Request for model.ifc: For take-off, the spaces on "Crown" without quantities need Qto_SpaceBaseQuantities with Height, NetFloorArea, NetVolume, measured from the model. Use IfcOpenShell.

First a look at what the model holds.

```python
import ifcopenshell
import ifcopenshell.util.element
import ifcopenshell.util.unit

model = ifcopenshell.open("model.ifc")
print(model.schema)
for unit_type in ("LENGTHUNIT", "AREAUNIT", "VOLUMEUNIT"):
    print(unit_type, ifcopenshell.util.unit.calculate_unit_scale(model, unit_type))
storey = next(s for s in model.by_type("IfcBuildingStorey") if s.Name == "Crown")
spaces = [e for e in ifcopenshell.util.element.get_decomposition(storey) if e.is_a("IfcSpace")]
for e in sorted(spaces, key=lambda e: e.id()):
    print(e.id(), e.is_a(), e.Name, list(ifcopenshell.util.element.get_psets(e, qtos_only=True)), sep=" | ")
```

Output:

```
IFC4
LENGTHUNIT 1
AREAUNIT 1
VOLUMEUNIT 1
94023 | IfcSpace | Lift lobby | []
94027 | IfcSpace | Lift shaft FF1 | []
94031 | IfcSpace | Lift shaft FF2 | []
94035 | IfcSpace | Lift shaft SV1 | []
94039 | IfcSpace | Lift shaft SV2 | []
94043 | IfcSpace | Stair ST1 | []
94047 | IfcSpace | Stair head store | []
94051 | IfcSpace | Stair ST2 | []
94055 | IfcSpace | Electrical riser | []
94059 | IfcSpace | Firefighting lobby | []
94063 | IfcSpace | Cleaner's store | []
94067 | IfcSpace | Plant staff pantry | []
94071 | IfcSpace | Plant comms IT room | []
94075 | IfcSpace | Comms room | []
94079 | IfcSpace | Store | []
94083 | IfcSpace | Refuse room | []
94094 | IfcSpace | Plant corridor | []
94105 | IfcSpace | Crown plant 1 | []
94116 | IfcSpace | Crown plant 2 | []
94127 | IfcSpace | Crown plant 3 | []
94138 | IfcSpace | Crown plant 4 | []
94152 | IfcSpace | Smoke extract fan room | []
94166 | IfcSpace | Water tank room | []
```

```python
import ifcopenshell
import ifcopenshell.api.pset
import ifcopenshell.geom
import ifcopenshell.util.element
import ifcopenshell.util.shape
import ifcopenshell.util.unit

model = ifcopenshell.open("model.ifc")
unit_scale = ifcopenshell.util.unit.calculate_unit_scale(model)
area_scale = ifcopenshell.util.unit.calculate_unit_scale(model, "AREAUNIT")
volume_scale = ifcopenshell.util.unit.calculate_unit_scale(model, "VOLUMEUNIT")
settings = ifcopenshell.geom.settings()

storey = next(s for s in model.by_type("IfcBuildingStorey") if s.Name == "Crown")
spaces = [e for e in ifcopenshell.util.element.get_decomposition(storey) if e.is_a("IfcSpace")]

for e in sorted(spaces, key=lambda e: e.id()):
    if ifcopenshell.util.element.get_psets(e, qtos_only=True, should_inherit=False):
        continue
    # Geometry comes back in metres, in the element's own axes.
    shape = ifcopenshell.geom.create_shape(settings, e)
    values = {
        "Height": ifcopenshell.util.shape.get_z(shape.geometry) / unit_scale,
        "NetFloorArea": ifcopenshell.util.shape.get_footprint_area(shape.geometry) / area_scale,
        "NetVolume": ifcopenshell.util.shape.get_volume(shape.geometry) / volume_scale,
    }
    qto = ifcopenshell.api.pset.add_qto(model, product=e, name="Qto_SpaceBaseQuantities")
    ifcopenshell.api.pset.edit_qto(model, qto=qto, properties=values)
    print(e.id(), {k: round(v, 3) for k, v in values.items()})

model.write("model_v2.ifc")
```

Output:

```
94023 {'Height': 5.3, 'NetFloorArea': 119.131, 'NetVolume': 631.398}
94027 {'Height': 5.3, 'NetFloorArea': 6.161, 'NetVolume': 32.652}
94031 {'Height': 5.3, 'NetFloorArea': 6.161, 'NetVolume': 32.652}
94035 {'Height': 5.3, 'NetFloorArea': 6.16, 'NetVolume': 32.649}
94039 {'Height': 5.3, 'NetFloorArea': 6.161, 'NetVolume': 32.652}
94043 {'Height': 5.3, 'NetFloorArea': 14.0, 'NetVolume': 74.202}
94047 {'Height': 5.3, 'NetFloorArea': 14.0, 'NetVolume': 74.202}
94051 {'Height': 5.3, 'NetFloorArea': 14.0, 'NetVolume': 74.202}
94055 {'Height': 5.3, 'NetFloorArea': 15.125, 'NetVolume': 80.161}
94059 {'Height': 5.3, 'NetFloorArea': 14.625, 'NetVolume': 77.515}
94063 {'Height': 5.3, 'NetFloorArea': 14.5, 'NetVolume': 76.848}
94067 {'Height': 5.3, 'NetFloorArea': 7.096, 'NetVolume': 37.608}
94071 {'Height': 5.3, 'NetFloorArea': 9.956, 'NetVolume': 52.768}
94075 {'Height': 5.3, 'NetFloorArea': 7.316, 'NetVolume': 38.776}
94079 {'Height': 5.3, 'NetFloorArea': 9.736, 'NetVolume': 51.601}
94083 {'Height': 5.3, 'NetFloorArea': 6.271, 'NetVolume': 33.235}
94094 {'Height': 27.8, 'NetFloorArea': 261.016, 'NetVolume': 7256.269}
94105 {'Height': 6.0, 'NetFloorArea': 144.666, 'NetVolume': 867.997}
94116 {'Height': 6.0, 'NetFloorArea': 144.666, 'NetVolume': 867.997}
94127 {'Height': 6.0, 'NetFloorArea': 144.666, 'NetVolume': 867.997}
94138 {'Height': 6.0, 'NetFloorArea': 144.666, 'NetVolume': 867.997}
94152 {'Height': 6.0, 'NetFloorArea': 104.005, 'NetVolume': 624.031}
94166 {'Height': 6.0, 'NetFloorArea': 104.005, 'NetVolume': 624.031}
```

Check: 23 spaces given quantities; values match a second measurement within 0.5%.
